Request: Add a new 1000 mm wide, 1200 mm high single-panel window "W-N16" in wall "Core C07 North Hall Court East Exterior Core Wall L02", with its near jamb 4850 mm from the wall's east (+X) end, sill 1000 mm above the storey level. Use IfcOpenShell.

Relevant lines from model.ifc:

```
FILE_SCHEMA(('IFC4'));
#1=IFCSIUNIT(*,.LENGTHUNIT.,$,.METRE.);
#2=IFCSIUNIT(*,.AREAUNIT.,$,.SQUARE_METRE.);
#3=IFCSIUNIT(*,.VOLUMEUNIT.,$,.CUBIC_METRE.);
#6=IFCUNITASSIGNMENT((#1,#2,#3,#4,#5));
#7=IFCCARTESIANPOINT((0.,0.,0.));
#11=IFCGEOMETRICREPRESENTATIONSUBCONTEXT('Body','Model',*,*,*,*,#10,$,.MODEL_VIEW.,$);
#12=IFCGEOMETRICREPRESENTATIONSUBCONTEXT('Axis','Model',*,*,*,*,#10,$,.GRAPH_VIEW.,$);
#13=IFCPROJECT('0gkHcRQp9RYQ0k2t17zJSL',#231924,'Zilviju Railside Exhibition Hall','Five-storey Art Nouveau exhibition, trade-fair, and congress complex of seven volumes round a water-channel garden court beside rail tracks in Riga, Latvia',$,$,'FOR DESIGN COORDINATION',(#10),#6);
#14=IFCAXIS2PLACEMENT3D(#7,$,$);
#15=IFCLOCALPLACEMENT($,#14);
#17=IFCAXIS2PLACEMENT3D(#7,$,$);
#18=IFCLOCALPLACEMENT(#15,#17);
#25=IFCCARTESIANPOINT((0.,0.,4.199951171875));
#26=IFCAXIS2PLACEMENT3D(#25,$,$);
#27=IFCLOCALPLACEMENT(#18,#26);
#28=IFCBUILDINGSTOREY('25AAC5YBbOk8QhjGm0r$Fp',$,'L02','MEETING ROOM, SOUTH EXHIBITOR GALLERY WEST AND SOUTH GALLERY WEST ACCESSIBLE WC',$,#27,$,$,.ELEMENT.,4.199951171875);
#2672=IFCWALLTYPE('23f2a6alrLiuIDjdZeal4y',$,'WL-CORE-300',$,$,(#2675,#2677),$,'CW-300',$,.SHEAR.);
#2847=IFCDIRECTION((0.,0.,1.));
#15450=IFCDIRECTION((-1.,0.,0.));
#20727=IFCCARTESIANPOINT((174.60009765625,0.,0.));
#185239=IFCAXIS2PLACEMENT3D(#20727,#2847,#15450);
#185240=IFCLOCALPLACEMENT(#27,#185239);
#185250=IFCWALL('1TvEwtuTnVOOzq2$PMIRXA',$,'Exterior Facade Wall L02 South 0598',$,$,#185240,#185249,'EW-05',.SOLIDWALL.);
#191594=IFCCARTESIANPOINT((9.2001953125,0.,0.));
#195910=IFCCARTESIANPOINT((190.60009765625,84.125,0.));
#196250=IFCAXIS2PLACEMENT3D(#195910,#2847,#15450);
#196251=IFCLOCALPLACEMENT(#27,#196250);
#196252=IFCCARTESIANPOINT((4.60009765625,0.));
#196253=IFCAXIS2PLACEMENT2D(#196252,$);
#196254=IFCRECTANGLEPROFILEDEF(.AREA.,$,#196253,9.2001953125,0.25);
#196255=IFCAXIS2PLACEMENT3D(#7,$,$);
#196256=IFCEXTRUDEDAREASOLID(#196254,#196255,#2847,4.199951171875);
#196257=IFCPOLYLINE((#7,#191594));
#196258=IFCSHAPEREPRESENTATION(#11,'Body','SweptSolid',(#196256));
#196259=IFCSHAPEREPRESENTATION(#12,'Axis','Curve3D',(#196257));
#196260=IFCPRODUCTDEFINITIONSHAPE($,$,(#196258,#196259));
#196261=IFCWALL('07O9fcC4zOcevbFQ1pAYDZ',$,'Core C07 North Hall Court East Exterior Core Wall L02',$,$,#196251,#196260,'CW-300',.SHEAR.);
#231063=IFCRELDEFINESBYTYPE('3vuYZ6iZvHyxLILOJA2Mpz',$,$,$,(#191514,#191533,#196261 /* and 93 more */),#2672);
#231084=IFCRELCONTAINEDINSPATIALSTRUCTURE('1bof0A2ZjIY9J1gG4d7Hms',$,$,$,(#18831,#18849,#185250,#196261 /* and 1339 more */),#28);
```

```python
import numpy as np
import ifcopenshell
import ifcopenshell.api.feature
import ifcopenshell.api.geometry
import ifcopenshell.api.root
import ifcopenshell.api.spatial
import ifcopenshell.geom
import ifcopenshell.util.element
import ifcopenshell.util.placement
import ifcopenshell.util.representation
import ifcopenshell.util.shape
import ifcopenshell.util.unit

model = ifcopenshell.open("model.ifc")
unit_scale = ifcopenshell.util.unit.calculate_unit_scale(model)
settings = ifcopenshell.geom.settings()


def volume(element):
    """Net volume in cubic metres, openings subtracted."""
    shape = ifcopenshell.geom.create_shape(settings, element)
    return ifcopenshell.util.shape.get_volume(shape.geometry)


wall = model.by_guid("07O9fcC4zOcevbFQ1pAYDZ")
storey = ifcopenshell.util.element.get_container(wall, ifc_class="IfcBuildingStorey")
context = ifcopenshell.util.representation.get_context(model, "Model", "Body", "MODEL_VIEW")
before = volume(wall)

width, height, from_end, sill = 1, 1.2, 4.85, 1  # metres

# The wall runs along its own X axis, and the end named is its -X end.
wall_shape = ifcopenshell.geom.create_shape(settings, wall)
x, y, z = ifcopenshell.util.shape.get_vertices(wall_shape.geometry).T
start = x.min() + from_end
face, thickness = float(y.min()), float(y.max() - y.min())
wall_matrix = ifcopenshell.util.placement.get_local_placement(wall.ObjectPlacement)
level = ifcopenshell.util.placement.get_local_placement(storey.ObjectPlacement)[2, 3]


def in_wall(x, y):
    """Placement at x, y metres in the wall's axes, at sill height."""
    matrix = wall_matrix.copy()
    matrix[:, 3] = wall_matrix @ np.array([x / unit_scale, y / unit_scale, 0.0, 1.0])
    matrix[2, 3] = level + sill / unit_scale
    return matrix


# Opening: a box that overshoots both wall faces by 50 mm.
opening = ifcopenshell.api.root.create_entity(model, ifc_class="IfcOpeningElement", predefined_type="OPENING")
box = ifcopenshell.api.geometry.add_wall_representation(
    model, context=context, length=width, height=height, thickness=thickness + 0.1
)
ifcopenshell.api.geometry.assign_representation(model, product=opening, representation=box)
ifcopenshell.api.geometry.edit_object_placement(model, product=opening, matrix=in_wall(start, face - 0.05), is_si=False)
ifcopenshell.api.feature.add_feature(model, feature=opening, element=wall)

window = ifcopenshell.api.root.create_entity(model, ifc_class="IfcWindow", name="W-N16", predefined_type="WINDOW")
window.OverallWidth, window.OverallHeight = width / unit_scale, height / unit_scale
window.PartitioningType = "SINGLE_PANEL"
body = ifcopenshell.api.geometry.add_window_representation(
    model,
    context=context,
    overall_width=window.OverallWidth,
    overall_height=window.OverallHeight,
    partition_type="SINGLE_PANEL",
)
ifcopenshell.api.geometry.assign_representation(model, product=window, representation=body)
ifcopenshell.api.spatial.assign_container(model, products=[window], relating_structure=storey)
ifcopenshell.api.feature.add_filling(model, opening=opening, element=window)

# Centre the window in the wall's thickness.
ifcopenshell.api.geometry.edit_object_placement(model, product=window, matrix=in_wall(start, face), is_si=False)
window_shape = ifcopenshell.geom.create_shape(settings, window)
depth = ifcopenshell.util.shape.get_vertices(window_shape.geometry)[:, 1]
offset = face + thickness / 2 - (depth.min() + depth.max()) / 2
ifcopenshell.api.geometry.edit_object_placement(model, product=window, matrix=in_wall(start, offset), is_si=False)

after = volume(wall)

print(f"wall volume {before:.3f} -> {after:.3f} m3")

model.write("model_v2.ifc")
```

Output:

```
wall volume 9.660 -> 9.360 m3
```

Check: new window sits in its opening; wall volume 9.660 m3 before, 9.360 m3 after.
